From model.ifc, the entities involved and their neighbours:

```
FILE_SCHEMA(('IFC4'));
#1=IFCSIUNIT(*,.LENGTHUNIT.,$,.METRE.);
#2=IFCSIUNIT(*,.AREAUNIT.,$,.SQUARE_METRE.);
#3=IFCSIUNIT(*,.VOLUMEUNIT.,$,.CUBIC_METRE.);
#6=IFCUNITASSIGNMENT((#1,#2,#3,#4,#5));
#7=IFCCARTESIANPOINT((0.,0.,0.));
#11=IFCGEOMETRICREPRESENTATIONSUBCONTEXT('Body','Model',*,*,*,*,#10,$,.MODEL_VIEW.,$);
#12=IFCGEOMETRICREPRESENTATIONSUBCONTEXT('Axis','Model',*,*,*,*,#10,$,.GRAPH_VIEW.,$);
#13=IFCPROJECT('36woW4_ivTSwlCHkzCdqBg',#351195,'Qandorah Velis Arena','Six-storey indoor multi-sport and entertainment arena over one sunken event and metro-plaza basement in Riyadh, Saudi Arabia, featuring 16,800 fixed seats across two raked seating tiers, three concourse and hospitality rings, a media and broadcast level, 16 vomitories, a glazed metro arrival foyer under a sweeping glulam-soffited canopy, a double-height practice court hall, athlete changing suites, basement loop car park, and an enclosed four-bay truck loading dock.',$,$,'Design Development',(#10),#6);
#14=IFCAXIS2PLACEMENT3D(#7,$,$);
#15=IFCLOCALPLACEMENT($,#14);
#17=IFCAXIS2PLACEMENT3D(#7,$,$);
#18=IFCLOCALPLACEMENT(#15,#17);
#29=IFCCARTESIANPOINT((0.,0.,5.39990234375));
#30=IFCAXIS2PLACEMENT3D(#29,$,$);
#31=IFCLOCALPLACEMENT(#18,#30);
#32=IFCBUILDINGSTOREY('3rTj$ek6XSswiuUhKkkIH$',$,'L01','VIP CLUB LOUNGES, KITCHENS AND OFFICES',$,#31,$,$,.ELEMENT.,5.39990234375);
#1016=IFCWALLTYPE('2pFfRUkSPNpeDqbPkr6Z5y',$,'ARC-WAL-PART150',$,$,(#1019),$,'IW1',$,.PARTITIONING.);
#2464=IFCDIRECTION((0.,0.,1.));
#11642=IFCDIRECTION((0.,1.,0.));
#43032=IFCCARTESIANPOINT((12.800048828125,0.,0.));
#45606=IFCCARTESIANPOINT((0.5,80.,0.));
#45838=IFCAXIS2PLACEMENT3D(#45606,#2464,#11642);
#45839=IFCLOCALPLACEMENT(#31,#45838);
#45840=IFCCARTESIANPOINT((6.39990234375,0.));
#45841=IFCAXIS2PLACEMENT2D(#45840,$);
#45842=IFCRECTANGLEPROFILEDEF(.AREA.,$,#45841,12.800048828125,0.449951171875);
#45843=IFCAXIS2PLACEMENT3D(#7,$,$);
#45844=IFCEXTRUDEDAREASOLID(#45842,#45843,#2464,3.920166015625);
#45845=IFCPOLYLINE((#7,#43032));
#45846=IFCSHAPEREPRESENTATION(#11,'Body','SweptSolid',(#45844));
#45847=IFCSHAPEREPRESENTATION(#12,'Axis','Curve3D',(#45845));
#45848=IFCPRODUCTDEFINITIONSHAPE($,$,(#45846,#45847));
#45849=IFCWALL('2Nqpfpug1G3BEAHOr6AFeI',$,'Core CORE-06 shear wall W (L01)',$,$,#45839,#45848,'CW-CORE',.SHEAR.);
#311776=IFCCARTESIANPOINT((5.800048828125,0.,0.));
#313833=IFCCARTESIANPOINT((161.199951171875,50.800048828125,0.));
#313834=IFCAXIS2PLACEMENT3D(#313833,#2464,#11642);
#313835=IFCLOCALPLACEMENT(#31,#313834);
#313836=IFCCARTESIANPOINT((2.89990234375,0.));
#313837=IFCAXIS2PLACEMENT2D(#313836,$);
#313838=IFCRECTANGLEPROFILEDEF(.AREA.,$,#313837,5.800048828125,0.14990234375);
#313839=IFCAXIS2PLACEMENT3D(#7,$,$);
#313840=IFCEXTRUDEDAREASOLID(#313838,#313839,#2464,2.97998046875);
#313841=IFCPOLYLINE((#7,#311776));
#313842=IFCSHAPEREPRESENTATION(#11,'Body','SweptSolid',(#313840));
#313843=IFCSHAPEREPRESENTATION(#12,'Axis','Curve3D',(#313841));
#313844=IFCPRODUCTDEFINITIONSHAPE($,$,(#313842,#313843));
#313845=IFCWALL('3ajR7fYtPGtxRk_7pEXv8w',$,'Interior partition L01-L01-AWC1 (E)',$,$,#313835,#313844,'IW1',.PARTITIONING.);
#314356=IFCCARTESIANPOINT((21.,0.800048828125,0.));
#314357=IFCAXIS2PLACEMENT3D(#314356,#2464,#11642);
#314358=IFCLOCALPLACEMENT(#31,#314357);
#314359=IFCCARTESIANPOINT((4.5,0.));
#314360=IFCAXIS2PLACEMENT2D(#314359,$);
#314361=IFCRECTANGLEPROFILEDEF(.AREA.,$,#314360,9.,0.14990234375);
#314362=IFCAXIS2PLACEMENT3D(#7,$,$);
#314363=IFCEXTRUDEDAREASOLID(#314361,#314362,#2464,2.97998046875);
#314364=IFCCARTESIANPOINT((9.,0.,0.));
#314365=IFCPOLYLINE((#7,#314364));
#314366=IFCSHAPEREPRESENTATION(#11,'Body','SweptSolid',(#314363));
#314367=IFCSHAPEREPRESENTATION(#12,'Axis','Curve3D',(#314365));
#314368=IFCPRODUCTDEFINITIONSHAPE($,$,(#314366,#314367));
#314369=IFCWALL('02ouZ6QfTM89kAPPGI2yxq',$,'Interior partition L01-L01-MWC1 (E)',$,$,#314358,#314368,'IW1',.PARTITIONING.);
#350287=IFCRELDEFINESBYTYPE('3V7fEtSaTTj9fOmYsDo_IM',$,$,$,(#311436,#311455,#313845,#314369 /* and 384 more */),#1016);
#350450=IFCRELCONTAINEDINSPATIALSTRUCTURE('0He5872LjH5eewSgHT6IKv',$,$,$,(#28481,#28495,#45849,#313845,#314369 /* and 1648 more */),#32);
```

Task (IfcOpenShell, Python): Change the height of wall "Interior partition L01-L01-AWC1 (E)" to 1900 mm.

```python
import ifcopenshell
import ifcopenshell.geom
import ifcopenshell.util.representation
import ifcopenshell.util.shape
import ifcopenshell.util.unit

model = ifcopenshell.open("model.ifc")
unit_scale = ifcopenshell.util.unit.calculate_unit_scale(model)
settings = ifcopenshell.geom.settings()


def volume(element):
    """Net volume in cubic metres, openings subtracted."""
    shape = ifcopenshell.geom.create_shape(settings, element)
    return ifcopenshell.util.shape.get_volume(shape.geometry)


wall = model.by_id(313845)
before = volume(wall)

body = ifcopenshell.util.representation.get_representation(wall, "Model", "Body")
solid = body.Items[0]
old_height = solid.Depth
solid.Depth = 1.9 / unit_scale
after = volume(wall)

print(f"height {old_height:g} -> {solid.Depth:g}, volume {before:.3f} -> {after:.3f} m3")

model.write("model-out.ifc")
```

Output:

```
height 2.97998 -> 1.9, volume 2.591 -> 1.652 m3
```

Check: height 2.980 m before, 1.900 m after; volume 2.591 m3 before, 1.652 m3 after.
